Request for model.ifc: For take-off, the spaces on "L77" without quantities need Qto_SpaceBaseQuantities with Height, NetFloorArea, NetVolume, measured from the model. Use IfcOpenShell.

First a look at what the model holds.

```python
import ifcopenshell
import ifcopenshell.util.element
import ifcopenshell.util.unit

model = ifcopenshell.open("model.ifc")
print(model.schema)
for unit_type in ("LENGTHUNIT", "AREAUNIT", "VOLUMEUNIT"):
    print(unit_type, ifcopenshell.util.unit.calculate_unit_scale(model, unit_type))
storey = next(s for s in model.by_type("IfcBuildingStorey") if s.Name == "L77")
spaces = [e for e in ifcopenshell.util.element.get_decomposition(storey) if e.is_a("IfcSpace")]
for e in sorted(spaces, key=lambda e: e.id()):
    print(e.id(), e.is_a(), e.Name, list(ifcopenshell.util.element.get_psets(e, qtos_only=True)), sep=" | ")
```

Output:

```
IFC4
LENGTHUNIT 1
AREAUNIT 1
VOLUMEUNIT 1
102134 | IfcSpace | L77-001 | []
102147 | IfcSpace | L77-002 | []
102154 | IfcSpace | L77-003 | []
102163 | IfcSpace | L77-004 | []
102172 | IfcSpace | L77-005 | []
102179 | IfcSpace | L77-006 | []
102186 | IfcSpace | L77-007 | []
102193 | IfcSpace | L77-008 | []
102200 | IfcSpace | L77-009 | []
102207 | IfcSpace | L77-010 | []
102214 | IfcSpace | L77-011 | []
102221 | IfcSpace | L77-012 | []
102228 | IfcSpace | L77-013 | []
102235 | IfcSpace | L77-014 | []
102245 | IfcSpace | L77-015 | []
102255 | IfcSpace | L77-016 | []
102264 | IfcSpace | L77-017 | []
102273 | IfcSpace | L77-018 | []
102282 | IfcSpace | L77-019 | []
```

```python
import ifcopenshell
import ifcopenshell.api.pset
import ifcopenshell.geom
import ifcopenshell.util.element
import ifcopenshell.util.shape
import ifcopenshell.util.unit

model = ifcopenshell.open("model.ifc")
unit_scale = ifcopenshell.util.unit.calculate_unit_scale(model)
area_scale = ifcopenshell.util.unit.calculate_unit_scale(model, "AREAUNIT")
volume_scale = ifcopenshell.util.unit.calculate_unit_scale(model, "VOLUMEUNIT")
settings = ifcopenshell.geom.settings()

storey = next(s for s in model.by_type("IfcBuildingStorey") if s.Name == "L77")
spaces = [e for e in ifcopenshell.util.element.get_decomposition(storey) if e.is_a("IfcSpace")]

for e in sorted(spaces, key=lambda e: e.id()):
    if ifcopenshell.util.element.get_psets(e, qtos_only=True, should_inherit=False):
        continue
    # Geometry comes back in metres, in the element's own axes.
    shape = ifcopenshell.geom.create_shape(settings, e)
    values = {
        "Height": ifcopenshell.util.shape.get_z(shape.geometry) / unit_scale,
        "NetFloorArea": ifcopenshell.util.shape.get_footprint_area(shape.geometry) / area_scale,
        "NetVolume": ifcopenshell.util.shape.get_volume(shape.geometry) / volume_scale,
    }
    qto = ifcopenshell.api.pset.add_qto(model, product=e, name="Qto_SpaceBaseQuantities")
    ifcopenshell.api.pset.edit_qto(model, qto=qto, properties=values)
    print(e.id(), {k: round(v, 3) for k, v in values.items()})

model.write("model_edited.ifc")
```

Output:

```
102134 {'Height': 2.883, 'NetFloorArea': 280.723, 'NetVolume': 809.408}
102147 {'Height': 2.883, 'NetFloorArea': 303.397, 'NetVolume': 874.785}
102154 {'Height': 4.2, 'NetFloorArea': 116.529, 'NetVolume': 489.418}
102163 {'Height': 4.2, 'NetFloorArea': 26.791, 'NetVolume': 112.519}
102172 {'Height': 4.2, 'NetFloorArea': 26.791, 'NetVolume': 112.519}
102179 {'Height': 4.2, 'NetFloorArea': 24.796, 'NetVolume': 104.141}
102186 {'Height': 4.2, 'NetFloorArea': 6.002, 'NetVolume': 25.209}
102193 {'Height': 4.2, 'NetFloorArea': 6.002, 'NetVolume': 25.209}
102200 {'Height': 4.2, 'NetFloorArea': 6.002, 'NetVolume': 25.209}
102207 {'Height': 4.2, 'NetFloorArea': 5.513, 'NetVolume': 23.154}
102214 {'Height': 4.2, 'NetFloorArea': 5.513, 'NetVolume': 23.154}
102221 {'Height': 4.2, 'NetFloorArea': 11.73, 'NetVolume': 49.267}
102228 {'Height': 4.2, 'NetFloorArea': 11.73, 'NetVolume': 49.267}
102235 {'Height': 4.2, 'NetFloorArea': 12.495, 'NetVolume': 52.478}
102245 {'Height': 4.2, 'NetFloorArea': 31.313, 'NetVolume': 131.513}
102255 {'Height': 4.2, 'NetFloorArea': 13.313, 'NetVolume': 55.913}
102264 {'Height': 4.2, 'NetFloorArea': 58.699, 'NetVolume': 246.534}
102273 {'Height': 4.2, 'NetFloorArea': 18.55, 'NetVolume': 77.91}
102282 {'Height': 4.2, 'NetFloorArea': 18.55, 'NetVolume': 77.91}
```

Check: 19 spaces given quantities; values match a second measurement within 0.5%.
